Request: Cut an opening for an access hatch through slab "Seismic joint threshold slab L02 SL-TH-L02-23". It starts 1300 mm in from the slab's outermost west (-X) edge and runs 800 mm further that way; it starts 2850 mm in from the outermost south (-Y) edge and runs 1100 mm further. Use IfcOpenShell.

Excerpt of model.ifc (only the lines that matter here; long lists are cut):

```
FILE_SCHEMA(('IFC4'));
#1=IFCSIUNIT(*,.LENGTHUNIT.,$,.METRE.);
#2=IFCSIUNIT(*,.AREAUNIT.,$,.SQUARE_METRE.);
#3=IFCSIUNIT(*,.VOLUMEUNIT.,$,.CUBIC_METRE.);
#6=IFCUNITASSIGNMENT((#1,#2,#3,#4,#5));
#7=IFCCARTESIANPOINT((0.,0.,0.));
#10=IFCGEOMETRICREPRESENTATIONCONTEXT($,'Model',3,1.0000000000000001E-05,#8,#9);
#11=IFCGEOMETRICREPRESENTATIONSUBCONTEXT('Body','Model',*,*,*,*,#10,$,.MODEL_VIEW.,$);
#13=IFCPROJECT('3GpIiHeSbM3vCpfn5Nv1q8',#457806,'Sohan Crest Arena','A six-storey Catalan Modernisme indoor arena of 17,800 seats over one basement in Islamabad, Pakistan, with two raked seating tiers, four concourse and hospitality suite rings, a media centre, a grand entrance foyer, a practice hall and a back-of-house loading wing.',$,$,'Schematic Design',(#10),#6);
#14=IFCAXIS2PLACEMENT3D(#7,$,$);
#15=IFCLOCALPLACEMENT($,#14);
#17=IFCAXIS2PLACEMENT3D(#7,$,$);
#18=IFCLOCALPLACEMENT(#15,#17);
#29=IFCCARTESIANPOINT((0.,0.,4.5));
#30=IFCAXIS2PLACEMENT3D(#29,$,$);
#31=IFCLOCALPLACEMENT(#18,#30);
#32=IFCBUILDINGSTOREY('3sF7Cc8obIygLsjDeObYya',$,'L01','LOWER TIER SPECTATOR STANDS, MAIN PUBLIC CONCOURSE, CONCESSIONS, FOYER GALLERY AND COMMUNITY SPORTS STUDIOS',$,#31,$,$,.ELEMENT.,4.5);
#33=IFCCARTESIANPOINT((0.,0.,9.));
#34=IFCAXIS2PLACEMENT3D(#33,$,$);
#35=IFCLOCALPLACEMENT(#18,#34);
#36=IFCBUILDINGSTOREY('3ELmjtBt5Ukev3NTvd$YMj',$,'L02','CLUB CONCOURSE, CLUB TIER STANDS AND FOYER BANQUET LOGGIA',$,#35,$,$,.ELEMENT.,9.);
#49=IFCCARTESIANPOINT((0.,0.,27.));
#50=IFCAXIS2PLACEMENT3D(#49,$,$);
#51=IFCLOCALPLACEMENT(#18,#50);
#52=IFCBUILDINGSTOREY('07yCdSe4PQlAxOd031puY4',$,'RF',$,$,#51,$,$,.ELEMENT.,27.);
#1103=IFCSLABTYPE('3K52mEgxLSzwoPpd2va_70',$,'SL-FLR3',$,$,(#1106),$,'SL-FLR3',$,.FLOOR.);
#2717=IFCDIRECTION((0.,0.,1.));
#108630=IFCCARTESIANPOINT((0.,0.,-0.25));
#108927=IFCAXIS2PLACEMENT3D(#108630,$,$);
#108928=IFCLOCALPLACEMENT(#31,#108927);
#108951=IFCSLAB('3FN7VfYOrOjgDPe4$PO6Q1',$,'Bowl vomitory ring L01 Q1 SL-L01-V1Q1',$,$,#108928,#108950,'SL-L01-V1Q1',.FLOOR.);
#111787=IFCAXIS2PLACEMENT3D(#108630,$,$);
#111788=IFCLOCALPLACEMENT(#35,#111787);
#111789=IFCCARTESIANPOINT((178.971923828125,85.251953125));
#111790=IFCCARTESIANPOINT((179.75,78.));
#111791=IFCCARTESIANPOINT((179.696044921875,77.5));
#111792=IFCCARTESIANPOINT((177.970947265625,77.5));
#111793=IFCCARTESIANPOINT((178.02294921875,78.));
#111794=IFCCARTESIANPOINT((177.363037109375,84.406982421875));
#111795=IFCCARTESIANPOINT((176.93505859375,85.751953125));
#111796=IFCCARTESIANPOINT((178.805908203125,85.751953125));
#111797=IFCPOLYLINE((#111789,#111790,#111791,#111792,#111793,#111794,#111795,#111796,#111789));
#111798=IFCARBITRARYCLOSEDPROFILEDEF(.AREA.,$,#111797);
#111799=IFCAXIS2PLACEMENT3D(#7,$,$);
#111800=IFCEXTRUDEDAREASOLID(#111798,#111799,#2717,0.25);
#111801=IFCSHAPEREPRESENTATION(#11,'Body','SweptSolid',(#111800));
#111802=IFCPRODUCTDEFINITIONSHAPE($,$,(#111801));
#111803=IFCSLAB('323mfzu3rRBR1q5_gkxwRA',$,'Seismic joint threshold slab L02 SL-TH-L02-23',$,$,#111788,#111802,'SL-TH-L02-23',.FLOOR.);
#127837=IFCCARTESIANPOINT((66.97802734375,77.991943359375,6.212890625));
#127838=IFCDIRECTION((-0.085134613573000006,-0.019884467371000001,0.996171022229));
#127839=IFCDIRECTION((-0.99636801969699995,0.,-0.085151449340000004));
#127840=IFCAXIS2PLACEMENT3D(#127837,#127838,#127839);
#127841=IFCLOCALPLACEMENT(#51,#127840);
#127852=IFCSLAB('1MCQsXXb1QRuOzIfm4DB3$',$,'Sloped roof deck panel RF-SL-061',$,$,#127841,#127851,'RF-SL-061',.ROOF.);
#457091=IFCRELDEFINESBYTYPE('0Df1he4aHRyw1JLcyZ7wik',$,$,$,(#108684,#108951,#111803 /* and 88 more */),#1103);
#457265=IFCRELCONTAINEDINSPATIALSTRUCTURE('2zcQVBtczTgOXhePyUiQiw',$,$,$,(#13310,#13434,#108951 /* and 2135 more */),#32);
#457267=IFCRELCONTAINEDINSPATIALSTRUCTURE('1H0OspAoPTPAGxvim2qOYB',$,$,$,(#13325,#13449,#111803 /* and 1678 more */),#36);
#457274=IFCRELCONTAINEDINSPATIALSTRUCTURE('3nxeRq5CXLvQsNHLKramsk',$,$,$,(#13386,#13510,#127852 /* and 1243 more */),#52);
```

```python
import numpy as np
import ifcopenshell
import ifcopenshell.api.feature
import ifcopenshell.api.geometry
import ifcopenshell.api.root
import ifcopenshell.geom
import ifcopenshell.util.placement
import ifcopenshell.util.representation
import ifcopenshell.util.shape
import ifcopenshell.util.unit

model = ifcopenshell.open("model.ifc")
unit_scale = ifcopenshell.util.unit.calculate_unit_scale(model)
settings = ifcopenshell.geom.settings()


def volume(element):
    """Net volume in cubic metres, openings subtracted."""
    shape = ifcopenshell.geom.create_shape(settings, element)
    return ifcopenshell.util.shape.get_volume(shape.geometry)


slab = model.by_guid("323mfzu3rRBR1q5_gkxwRA")
before = volume(slab)

# Extent in the slab's own axes, in metres. The edges named are its -X and -Y sides.
slab_shape = ifcopenshell.geom.create_shape(settings, slab)
vertices = ifcopenshell.util.shape.get_vertices(slab_shape.geometry)
x_min, y_min, bottom = vertices.min(axis=0)
top = vertices[:, 2].max()

opening = ifcopenshell.api.root.create_entity(model, ifc_class="IfcOpeningElement", name="Access hatch opening", predefined_type="OPENING")
context = ifcopenshell.util.representation.get_context(model, "Model", "Body", "MODEL_VIEW")
width, depth = 0.8, 1.1
outline = [(0.0, 0.0), (width, 0.0), (width, depth), (0.0, depth), (0.0, 0.0)]
# Overshoot both faces by 50 mm so the cut is clean.
shape = ifcopenshell.api.geometry.add_slab_representation(
    model, context=context, depth=top - bottom + 0.1, polyline=outline
)
ifcopenshell.api.geometry.assign_representation(model, product=opening, representation=shape)

matrix = ifcopenshell.util.placement.get_local_placement(slab.ObjectPlacement)
matrix[:, 3] = matrix @ np.append(np.array([x_min + 1.3, y_min + 2.85, bottom - 0.05]) / unit_scale, 1.0)
ifcopenshell.api.geometry.edit_object_placement(model, product=opening, matrix=matrix, is_si=False)
ifcopenshell.api.feature.add_feature(model, feature=opening, element=slab)

after = volume(slab)

print(f"slab volume {before:.3f} -> {after:.3f} m3")

model.write("model_updated.ifc")
```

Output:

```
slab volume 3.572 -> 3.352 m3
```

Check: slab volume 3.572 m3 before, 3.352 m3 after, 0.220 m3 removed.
